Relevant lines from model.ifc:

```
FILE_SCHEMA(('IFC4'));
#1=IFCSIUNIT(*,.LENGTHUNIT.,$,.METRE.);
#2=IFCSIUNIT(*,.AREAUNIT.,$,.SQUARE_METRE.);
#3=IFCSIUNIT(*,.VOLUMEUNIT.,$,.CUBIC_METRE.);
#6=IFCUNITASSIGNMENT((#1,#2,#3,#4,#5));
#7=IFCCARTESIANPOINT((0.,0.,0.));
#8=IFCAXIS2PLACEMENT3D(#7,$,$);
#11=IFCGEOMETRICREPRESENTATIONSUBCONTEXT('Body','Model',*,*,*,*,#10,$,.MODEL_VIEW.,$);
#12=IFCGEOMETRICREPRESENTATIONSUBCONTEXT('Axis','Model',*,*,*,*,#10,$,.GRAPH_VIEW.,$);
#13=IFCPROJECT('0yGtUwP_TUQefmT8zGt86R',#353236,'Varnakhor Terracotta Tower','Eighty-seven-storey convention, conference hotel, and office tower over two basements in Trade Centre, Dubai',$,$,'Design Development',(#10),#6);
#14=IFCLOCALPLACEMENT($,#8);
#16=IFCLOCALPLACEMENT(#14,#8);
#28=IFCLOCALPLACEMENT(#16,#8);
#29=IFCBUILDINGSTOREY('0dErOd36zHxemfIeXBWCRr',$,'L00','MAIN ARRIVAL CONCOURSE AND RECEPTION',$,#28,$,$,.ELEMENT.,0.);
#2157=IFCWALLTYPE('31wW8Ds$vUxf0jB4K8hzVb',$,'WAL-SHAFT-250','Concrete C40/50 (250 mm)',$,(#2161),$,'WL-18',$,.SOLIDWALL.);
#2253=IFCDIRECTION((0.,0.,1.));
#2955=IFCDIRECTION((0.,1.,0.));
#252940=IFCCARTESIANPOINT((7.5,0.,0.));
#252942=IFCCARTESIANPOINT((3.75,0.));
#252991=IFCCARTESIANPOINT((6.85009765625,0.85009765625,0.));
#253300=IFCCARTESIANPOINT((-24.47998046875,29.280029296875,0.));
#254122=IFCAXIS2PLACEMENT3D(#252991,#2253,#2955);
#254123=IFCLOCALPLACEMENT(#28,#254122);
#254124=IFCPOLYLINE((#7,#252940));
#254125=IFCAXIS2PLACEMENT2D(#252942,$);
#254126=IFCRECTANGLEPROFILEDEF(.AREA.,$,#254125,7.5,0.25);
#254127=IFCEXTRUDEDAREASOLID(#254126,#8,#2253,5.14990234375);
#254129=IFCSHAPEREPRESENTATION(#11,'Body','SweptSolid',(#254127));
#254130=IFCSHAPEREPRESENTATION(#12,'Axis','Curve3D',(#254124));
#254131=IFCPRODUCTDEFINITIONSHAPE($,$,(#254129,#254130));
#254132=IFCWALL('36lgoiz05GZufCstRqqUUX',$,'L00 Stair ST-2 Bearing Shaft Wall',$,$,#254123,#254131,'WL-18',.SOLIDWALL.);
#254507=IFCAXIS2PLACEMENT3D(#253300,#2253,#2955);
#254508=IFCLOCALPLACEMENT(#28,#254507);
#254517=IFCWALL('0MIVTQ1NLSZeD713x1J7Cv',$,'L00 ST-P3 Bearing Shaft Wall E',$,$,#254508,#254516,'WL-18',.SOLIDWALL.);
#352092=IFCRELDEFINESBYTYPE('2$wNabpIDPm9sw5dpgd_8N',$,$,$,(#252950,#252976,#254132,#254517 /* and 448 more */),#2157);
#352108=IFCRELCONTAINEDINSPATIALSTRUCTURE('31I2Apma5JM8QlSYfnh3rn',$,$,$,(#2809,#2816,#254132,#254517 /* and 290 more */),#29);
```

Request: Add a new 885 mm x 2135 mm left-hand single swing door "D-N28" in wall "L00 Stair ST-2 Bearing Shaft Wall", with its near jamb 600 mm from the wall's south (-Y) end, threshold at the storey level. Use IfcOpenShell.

```python
import numpy as np
import ifcopenshell
import ifcopenshell.api.feature
import ifcopenshell.api.geometry
import ifcopenshell.api.root
import ifcopenshell.api.spatial
import ifcopenshell.geom
import ifcopenshell.util.element
import ifcopenshell.util.placement
import ifcopenshell.util.representation
import ifcopenshell.util.shape
import ifcopenshell.util.unit

model = ifcopenshell.open("model.ifc")
unit_scale = ifcopenshell.util.unit.calculate_unit_scale(model)
settings = ifcopenshell.geom.settings()


def volume(element):
    """Net volume in cubic metres, openings subtracted."""
    shape = ifcopenshell.geom.create_shape(settings, element)
    return ifcopenshell.util.shape.get_volume(shape.geometry)


wall = model.by_guid("36lgoiz05GZufCstRqqUUX")
storey = ifcopenshell.util.element.get_container(wall, ifc_class="IfcBuildingStorey")
context = ifcopenshell.util.representation.get_context(model, "Model", "Body", "MODEL_VIEW")
before = volume(wall)

width, height, from_end, sill = 0.885, 2.135, 0.6, 0.0  # metres

# The wall runs along its own X axis, and the end named is its -X end.
wall_shape = ifcopenshell.geom.create_shape(settings, wall)
x, y, z = ifcopenshell.util.shape.get_vertices(wall_shape.geometry).T
start = x.min() + from_end
face, thickness = float(y.min()), float(y.max() - y.min())
wall_matrix = ifcopenshell.util.placement.get_local_placement(wall.ObjectPlacement)
level = ifcopenshell.util.placement.get_local_placement(storey.ObjectPlacement)[2, 3]


def in_wall(x, y):
    """Placement at x, y metres in the wall's axes, at sill height."""
    matrix = wall_matrix.copy()
    matrix[:, 3] = wall_matrix @ np.array([x / unit_scale, y / unit_scale, 0.0, 1.0])
    matrix[2, 3] = level + sill / unit_scale
    return matrix


# Opening: a box that overshoots both wall faces by 50 mm.
opening = ifcopenshell.api.root.create_entity(model, ifc_class="IfcOpeningElement", predefined_type="OPENING")
box = ifcopenshell.api.geometry.add_wall_representation(
    model, context=context, length=width, height=height, thickness=thickness + 0.1
)
ifcopenshell.api.geometry.assign_representation(model, product=opening, representation=box)
ifcopenshell.api.geometry.edit_object_placement(model, product=opening, matrix=in_wall(start, face - 0.05), is_si=False)
ifcopenshell.api.feature.add_feature(model, feature=opening, element=wall)

door = ifcopenshell.api.root.create_entity(model, ifc_class="IfcDoor", name="D-N28", predefined_type="DOOR")
door.OverallWidth, door.OverallHeight = width / unit_scale, height / unit_scale
door.OperationType = "SINGLE_SWING_LEFT"
body = ifcopenshell.api.geometry.add_door_representation(
    model,
    context=context,
    overall_width=door.OverallWidth,
    overall_height=door.OverallHeight,
    operation_type="SINGLE_SWING_LEFT",
    lining_properties={"LiningDepth": thickness / unit_scale, "ThresholdDepth": thickness / unit_scale},
)
ifcopenshell.api.geometry.assign_representation(model, product=door, representation=body)
ifcopenshell.api.spatial.assign_container(model, products=[door], relating_structure=storey)
ifcopenshell.api.feature.add_filling(model, opening=opening, element=door)

# The lining spans the wall, so the door starts at the wall face.
ifcopenshell.api.geometry.edit_object_placement(model, product=door, matrix=in_wall(start, face), is_si=False)

after = volume(wall)

print(f"wall volume {before:.3f} -> {after:.3f} m3")

model.write("model_updated.ifc")
```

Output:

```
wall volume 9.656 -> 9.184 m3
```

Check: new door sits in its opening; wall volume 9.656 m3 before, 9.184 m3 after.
